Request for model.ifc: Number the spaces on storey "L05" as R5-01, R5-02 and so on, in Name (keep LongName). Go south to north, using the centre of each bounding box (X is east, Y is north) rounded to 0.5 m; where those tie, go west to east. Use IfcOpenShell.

First a look at what the model holds.

```python
import ifcopenshell
import ifcopenshell.util.element
import ifcopenshell.util.placement

model = ifcopenshell.open("model.ifc")
print(model.schema)
storey = next(s for s in model.by_type("IfcBuildingStorey") if s.Name == "L05")
spaces = [e for e in ifcopenshell.util.element.get_decomposition(storey) if e.is_a("IfcSpace")]
for e in sorted(spaces, key=lambda e: e.id()):
    origin = ifcopenshell.util.placement.get_local_placement(e.ObjectPlacement)[:3, 3]
    print(e.id(), e.Name, e.LongName, origin.round(2) + 0.0, sep=" | ")
```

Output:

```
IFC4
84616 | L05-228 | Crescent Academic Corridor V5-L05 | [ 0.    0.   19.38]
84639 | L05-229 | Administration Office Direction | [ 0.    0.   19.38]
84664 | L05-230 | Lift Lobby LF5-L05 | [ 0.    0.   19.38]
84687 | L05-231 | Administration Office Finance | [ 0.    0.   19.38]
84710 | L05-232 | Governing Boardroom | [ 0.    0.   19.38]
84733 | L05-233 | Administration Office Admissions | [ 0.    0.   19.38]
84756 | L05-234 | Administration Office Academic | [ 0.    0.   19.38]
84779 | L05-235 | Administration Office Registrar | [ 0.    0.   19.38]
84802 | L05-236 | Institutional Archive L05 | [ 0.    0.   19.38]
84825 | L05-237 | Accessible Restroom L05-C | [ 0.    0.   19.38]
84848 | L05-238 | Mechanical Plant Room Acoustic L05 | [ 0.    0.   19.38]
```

```python
import ifcopenshell
import ifcopenshell.geom
import ifcopenshell.util.element
import ifcopenshell.util.shape

model = ifcopenshell.open("model.ifc")
settings = ifcopenshell.geom.settings()
settings.set("use-world-coords", True)


def centre(element):
    shape = ifcopenshell.geom.create_shape(settings, element)
    return ifcopenshell.util.shape.get_bbox_centroid(shape.geometry)


storey = next(s for s in model.by_type("IfcBuildingStorey") if s.Name == "L05")
spaces = [e for e in ifcopenshell.util.element.get_decomposition(storey) if e.is_a("IfcSpace")]

# Insertion points can sit at a corner or the storey origin, so sort by the geometry (in metres).
centres = {e: centre(e) for e in spaces}
spaces.sort(key=lambda e: (round(centres[e][1] / 0.5), centres[e][0]))

for i, e in enumerate(spaces, start=1):
    number = f"R5-{i:02d}"
    e.Name = number
    print(e.id(), number)

model.write("model_v2.ifc")
```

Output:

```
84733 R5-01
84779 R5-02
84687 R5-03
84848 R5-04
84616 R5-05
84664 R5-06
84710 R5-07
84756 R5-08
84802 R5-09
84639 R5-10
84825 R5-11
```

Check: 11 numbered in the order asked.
